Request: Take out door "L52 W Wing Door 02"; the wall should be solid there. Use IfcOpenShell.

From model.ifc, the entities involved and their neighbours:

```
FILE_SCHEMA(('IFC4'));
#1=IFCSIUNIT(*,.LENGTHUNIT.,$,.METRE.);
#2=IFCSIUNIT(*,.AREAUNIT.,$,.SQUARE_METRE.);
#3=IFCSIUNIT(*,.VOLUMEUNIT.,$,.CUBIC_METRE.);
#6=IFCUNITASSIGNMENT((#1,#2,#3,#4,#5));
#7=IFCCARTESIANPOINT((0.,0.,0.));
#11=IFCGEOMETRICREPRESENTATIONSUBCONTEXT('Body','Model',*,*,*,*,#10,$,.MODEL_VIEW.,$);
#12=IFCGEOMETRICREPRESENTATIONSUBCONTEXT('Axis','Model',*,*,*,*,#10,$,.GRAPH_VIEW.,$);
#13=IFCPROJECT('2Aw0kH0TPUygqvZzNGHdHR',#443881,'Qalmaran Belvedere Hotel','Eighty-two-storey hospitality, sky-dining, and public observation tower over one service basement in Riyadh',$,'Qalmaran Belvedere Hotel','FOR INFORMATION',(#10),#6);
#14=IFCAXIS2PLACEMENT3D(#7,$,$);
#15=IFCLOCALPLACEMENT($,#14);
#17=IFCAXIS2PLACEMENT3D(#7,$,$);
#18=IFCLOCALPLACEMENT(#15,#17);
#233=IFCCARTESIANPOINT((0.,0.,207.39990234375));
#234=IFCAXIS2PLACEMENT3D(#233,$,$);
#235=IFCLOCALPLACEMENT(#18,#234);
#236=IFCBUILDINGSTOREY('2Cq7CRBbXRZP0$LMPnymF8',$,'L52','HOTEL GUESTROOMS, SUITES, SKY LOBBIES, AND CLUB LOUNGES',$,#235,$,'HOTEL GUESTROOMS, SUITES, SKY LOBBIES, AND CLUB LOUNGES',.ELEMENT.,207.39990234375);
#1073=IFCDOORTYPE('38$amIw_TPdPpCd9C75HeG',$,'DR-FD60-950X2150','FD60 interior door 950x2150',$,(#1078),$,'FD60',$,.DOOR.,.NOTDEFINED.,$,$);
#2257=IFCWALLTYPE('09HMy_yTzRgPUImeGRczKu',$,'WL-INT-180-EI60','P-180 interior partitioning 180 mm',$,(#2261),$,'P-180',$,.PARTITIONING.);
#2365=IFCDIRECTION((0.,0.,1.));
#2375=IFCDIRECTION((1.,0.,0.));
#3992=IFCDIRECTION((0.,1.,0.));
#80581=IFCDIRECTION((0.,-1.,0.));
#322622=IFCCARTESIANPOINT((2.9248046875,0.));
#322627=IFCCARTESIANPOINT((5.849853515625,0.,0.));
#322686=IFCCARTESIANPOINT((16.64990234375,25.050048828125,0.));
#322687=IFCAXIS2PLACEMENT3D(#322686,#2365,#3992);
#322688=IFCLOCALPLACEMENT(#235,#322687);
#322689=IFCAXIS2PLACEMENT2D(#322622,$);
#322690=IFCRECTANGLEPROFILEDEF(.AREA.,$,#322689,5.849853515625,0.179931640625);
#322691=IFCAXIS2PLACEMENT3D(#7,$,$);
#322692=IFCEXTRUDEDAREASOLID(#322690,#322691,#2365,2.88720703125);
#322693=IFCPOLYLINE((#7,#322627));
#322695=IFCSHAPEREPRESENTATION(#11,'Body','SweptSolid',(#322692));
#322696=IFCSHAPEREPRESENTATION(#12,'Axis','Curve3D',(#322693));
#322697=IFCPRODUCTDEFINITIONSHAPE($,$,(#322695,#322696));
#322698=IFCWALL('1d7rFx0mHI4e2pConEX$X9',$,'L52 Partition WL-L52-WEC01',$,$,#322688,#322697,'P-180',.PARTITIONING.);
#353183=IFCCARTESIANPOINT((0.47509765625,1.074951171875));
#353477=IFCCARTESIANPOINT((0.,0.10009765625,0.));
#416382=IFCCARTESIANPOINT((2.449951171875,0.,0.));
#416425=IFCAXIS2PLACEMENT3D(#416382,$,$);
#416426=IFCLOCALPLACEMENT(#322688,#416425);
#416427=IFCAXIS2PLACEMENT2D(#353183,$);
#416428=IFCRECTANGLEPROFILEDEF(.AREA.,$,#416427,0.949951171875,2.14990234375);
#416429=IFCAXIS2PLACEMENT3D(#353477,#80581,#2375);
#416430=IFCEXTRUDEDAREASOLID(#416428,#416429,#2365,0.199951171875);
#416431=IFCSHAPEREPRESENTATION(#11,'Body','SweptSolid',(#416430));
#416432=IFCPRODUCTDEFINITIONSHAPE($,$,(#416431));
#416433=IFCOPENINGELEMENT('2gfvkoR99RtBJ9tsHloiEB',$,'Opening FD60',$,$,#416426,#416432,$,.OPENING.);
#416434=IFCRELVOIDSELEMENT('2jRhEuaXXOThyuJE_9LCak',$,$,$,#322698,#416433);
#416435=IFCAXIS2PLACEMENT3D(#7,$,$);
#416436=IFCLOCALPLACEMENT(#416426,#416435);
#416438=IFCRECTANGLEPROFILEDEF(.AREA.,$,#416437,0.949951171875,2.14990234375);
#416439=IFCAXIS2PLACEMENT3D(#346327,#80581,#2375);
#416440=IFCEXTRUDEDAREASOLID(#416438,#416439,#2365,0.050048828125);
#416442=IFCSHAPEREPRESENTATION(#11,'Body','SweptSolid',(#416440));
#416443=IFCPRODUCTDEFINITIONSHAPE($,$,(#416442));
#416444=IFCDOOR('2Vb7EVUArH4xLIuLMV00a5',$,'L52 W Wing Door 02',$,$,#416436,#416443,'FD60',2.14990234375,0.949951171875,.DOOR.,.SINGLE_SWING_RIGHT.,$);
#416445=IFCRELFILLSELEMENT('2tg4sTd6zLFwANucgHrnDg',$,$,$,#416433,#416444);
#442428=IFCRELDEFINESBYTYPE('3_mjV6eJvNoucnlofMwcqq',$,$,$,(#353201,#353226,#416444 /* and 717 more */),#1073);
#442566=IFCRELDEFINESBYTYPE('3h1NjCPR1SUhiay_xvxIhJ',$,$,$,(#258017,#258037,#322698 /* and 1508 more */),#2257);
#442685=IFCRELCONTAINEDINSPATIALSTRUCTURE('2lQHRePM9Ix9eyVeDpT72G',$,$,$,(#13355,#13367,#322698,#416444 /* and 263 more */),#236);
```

```python
import ifcopenshell
import ifcopenshell.api.feature
import ifcopenshell.api.root
import ifcopenshell.geom
import ifcopenshell.util.shape

model = ifcopenshell.open("model.ifc")
settings = ifcopenshell.geom.settings()


def volume(element):
    """Net volume in cubic metres, openings subtracted."""
    shape = ifcopenshell.geom.create_shape(settings, element)
    return ifcopenshell.util.shape.get_volume(shape.geometry)


door = model.by_guid("2Vb7EVUArH4xLIuLMV00a5")
opening = door.FillsVoids[0].RelatingOpeningElement
wall = opening.VoidsElements[0].RelatingBuildingElement
before = volume(wall)

ifcopenshell.api.root.remove_product(model, product=door)
ifcopenshell.api.feature.remove_feature(model, feature=opening)

after = volume(wall)

print(f"wall volume {before:.3f} -> {after:.3f} m3")

model.write("model-out.ifc")
```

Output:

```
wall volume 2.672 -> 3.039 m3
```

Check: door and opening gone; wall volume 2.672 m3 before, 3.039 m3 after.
